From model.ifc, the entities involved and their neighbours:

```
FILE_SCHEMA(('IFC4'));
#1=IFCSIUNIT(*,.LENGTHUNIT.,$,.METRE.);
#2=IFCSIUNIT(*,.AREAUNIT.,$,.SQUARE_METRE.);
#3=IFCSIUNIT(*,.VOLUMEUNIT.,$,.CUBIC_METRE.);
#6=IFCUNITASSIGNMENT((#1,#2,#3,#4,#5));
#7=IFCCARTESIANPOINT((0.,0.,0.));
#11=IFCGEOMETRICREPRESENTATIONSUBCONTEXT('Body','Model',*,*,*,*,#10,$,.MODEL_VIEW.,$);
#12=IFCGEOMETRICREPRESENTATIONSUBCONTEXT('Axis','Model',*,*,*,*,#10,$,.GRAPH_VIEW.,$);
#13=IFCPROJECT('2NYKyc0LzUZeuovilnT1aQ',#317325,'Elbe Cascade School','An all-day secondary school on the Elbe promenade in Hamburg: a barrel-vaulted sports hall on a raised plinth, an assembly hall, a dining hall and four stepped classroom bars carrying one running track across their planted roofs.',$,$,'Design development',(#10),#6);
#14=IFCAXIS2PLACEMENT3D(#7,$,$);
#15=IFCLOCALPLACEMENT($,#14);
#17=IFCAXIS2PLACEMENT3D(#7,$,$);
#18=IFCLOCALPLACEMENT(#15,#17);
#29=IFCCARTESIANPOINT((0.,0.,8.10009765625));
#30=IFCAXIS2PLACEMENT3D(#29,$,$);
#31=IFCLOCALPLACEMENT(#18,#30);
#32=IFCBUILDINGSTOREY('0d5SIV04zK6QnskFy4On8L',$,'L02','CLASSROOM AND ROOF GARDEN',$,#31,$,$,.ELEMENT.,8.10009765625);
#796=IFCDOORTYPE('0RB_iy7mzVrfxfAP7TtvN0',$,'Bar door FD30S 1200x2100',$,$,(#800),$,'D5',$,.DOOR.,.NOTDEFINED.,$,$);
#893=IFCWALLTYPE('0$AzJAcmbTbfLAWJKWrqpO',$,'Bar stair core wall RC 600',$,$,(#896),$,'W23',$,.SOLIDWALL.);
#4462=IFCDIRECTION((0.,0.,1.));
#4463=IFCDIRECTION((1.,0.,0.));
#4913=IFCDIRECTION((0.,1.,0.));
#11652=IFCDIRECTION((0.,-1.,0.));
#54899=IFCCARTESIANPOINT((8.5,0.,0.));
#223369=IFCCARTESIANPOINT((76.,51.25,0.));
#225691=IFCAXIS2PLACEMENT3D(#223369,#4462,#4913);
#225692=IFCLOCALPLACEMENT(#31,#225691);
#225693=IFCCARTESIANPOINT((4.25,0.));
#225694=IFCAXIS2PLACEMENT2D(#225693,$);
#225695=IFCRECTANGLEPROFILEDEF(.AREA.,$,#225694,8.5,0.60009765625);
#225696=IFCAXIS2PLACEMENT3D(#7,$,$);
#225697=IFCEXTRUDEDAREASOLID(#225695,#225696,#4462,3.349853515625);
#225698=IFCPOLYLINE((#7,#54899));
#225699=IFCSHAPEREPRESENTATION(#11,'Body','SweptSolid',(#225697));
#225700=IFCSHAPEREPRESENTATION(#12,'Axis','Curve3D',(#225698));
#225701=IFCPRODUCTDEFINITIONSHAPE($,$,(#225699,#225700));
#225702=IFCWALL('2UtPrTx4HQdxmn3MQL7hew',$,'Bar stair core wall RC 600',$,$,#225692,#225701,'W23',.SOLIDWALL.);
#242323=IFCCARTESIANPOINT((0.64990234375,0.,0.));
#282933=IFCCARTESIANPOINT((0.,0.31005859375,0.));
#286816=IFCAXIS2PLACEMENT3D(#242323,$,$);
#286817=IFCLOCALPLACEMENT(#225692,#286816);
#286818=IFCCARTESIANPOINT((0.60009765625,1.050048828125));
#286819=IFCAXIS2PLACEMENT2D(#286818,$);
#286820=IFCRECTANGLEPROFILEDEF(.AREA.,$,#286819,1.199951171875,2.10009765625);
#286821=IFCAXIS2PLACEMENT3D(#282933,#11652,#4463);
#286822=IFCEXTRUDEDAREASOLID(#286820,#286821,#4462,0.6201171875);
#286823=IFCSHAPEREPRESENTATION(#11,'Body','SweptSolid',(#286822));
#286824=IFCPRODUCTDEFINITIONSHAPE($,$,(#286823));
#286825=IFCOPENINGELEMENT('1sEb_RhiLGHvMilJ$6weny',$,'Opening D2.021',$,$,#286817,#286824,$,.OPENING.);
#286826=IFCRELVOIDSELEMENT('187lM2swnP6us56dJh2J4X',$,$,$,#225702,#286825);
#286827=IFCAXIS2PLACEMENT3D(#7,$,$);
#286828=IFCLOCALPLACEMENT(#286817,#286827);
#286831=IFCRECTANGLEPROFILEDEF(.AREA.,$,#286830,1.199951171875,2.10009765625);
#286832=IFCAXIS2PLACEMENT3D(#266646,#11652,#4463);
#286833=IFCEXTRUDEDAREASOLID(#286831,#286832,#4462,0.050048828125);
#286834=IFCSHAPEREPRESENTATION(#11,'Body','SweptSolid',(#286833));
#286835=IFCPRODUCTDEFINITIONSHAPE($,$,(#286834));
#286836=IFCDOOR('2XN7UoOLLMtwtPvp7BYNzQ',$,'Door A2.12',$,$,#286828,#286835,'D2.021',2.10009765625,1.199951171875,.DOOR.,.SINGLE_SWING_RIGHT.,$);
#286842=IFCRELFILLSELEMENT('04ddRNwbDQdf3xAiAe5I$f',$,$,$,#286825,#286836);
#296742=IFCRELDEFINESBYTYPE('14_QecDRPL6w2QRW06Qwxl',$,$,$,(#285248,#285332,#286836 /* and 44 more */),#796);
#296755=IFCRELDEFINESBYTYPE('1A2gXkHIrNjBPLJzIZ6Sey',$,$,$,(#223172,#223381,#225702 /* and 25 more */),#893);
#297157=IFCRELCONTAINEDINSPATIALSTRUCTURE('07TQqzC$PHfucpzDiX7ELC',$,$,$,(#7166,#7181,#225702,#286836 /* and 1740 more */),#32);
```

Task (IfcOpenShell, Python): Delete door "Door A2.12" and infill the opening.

```python
import ifcopenshell
import ifcopenshell.api.feature
import ifcopenshell.api.root
import ifcopenshell.geom
import ifcopenshell.util.shape

model = ifcopenshell.open("model.ifc")
settings = ifcopenshell.geom.settings()


def volume(element):
    """Net volume in cubic metres, openings subtracted."""
    shape = ifcopenshell.geom.create_shape(settings, element)
    return ifcopenshell.util.shape.get_volume(shape.geometry)


door = model.by_guid("2XN7UoOLLMtwtPvp7BYNzQ")
opening = door.FillsVoids[0].RelatingOpeningElement
wall = opening.VoidsElements[0].RelatingBuildingElement
before = volume(wall)

ifcopenshell.api.root.remove_product(model, product=door)
ifcopenshell.api.feature.remove_feature(model, feature=opening)

after = volume(wall)

print(f"wall volume {before:.3f} -> {after:.3f} m3")

model.write("model-out.ifc")
```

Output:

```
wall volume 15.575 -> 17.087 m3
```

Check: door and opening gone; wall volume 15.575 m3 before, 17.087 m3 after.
